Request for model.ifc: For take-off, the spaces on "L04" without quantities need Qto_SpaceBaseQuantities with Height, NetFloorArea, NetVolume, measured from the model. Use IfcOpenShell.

First a look at what the model holds.

```python
import ifcopenshell
import ifcopenshell.util.element
import ifcopenshell.util.unit

model = ifcopenshell.open("model.ifc")
print(model.schema)
for unit_type in ("LENGTHUNIT", "AREAUNIT", "VOLUMEUNIT"):
    print(unit_type, ifcopenshell.util.unit.calculate_unit_scale(model, unit_type))
storey = next(s for s in model.by_type("IfcBuildingStorey") if s.Name == "L04")
spaces = [e for e in ifcopenshell.util.element.get_decomposition(storey) if e.is_a("IfcSpace")]
for e in sorted(spaces, key=lambda e: e.id()):
    print(e.id(), e.is_a(), e.Name, list(ifcopenshell.util.element.get_psets(e, qtos_only=True)), sep=" | ")
```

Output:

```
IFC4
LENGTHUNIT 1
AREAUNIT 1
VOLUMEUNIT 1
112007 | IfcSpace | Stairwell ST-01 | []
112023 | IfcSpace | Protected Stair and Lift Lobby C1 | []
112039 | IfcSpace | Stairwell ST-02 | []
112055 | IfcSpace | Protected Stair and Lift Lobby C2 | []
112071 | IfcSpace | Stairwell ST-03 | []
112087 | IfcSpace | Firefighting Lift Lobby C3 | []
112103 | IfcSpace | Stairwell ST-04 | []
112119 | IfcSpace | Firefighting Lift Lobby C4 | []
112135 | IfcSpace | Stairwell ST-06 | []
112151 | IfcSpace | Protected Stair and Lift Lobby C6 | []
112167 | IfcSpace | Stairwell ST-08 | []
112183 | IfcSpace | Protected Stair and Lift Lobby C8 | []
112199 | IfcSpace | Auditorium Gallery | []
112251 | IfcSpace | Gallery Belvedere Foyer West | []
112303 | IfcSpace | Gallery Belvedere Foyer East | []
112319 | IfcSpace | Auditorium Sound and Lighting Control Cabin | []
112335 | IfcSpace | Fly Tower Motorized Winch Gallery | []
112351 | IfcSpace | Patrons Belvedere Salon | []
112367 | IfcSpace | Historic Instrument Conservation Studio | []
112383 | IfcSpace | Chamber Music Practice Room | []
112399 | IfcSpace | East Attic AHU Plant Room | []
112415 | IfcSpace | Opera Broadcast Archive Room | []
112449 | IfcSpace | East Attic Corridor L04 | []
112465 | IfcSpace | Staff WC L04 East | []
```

```python
import ifcopenshell
import ifcopenshell.api.pset
import ifcopenshell.geom
import ifcopenshell.util.element
import ifcopenshell.util.shape
import ifcopenshell.util.unit

model = ifcopenshell.open("model.ifc")
unit_scale = ifcopenshell.util.unit.calculate_unit_scale(model)
area_scale = ifcopenshell.util.unit.calculate_unit_scale(model, "AREAUNIT")
volume_scale = ifcopenshell.util.unit.calculate_unit_scale(model, "VOLUMEUNIT")
settings = ifcopenshell.geom.settings()

storey = next(s for s in model.by_type("IfcBuildingStorey") if s.Name == "L04")
spaces = [e for e in ifcopenshell.util.element.get_decomposition(storey) if e.is_a("IfcSpace")]

for e in sorted(spaces, key=lambda e: e.id()):
    if ifcopenshell.util.element.get_psets(e, qtos_only=True, should_inherit=False):
        continue
    # Geometry comes back in metres, in the element's own axes.
    shape = ifcopenshell.geom.create_shape(settings, e)
    values = {
        "Height": ifcopenshell.util.shape.get_z(shape.geometry) / unit_scale,
        "NetFloorArea": ifcopenshell.util.shape.get_footprint_area(shape.geometry) / area_scale,
        "NetVolume": ifcopenshell.util.shape.get_volume(shape.geometry) / volume_scale,
    }
    qto = ifcopenshell.api.pset.add_qto(model, product=e, name="Qto_SpaceBaseQuantities")
    ifcopenshell.api.pset.edit_qto(model, qto=qto, properties=values)
    print(e.id(), {k: round(v, 3) for k, v in values.items()})

model.write("model-out.ifc")
```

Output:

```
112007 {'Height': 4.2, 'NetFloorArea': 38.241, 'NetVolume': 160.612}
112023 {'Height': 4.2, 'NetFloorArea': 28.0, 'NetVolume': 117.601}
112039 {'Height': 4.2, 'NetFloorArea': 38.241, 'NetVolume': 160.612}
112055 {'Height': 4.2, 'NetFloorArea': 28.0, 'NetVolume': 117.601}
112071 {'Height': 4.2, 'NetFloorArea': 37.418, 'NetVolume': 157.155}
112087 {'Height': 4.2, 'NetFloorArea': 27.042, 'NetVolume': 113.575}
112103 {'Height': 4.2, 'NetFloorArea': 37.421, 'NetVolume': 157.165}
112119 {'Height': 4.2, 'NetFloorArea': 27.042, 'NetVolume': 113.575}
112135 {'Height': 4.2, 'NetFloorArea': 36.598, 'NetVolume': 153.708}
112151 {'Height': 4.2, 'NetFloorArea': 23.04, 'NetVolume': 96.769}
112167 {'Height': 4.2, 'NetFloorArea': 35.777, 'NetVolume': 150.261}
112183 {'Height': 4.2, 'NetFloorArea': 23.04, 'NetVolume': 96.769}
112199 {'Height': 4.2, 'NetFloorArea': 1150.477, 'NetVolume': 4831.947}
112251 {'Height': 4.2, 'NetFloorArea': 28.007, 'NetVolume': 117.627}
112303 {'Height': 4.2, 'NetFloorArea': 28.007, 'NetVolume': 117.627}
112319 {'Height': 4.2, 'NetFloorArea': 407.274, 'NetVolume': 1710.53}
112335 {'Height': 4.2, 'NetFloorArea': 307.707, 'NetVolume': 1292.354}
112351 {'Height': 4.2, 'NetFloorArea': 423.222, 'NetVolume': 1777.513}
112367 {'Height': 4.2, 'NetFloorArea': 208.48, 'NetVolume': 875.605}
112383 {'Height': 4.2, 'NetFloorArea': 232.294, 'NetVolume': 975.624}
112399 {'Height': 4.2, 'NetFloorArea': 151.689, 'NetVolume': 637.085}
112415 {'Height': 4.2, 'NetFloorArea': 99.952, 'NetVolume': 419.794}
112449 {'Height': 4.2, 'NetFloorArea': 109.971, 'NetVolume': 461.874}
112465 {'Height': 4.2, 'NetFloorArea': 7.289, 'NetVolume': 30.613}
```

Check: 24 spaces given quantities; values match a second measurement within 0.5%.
